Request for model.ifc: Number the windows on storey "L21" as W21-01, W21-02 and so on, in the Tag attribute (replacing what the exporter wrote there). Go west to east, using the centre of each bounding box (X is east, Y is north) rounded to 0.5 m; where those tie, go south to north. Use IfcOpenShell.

First a look at what the model holds.

```python
import ifcopenshell
import ifcopenshell.util.element
import ifcopenshell.util.placement

model = ifcopenshell.open("model.ifc")
print(model.schema)
storey = next(s for s in model.by_type("IfcBuildingStorey") if s.Name == "L21")
windows = [e for e in ifcopenshell.util.element.get_decomposition(storey) if e.is_a("IfcWindow")]
for e in sorted(windows, key=lambda e: e.id()):
    origin = ifcopenshell.util.placement.get_local_placement(e.ObjectPlacement)[:3, 3]
    print(e.id(), e.Tag, e.Name, origin.round(2) + 0.0, sep=" | ")
```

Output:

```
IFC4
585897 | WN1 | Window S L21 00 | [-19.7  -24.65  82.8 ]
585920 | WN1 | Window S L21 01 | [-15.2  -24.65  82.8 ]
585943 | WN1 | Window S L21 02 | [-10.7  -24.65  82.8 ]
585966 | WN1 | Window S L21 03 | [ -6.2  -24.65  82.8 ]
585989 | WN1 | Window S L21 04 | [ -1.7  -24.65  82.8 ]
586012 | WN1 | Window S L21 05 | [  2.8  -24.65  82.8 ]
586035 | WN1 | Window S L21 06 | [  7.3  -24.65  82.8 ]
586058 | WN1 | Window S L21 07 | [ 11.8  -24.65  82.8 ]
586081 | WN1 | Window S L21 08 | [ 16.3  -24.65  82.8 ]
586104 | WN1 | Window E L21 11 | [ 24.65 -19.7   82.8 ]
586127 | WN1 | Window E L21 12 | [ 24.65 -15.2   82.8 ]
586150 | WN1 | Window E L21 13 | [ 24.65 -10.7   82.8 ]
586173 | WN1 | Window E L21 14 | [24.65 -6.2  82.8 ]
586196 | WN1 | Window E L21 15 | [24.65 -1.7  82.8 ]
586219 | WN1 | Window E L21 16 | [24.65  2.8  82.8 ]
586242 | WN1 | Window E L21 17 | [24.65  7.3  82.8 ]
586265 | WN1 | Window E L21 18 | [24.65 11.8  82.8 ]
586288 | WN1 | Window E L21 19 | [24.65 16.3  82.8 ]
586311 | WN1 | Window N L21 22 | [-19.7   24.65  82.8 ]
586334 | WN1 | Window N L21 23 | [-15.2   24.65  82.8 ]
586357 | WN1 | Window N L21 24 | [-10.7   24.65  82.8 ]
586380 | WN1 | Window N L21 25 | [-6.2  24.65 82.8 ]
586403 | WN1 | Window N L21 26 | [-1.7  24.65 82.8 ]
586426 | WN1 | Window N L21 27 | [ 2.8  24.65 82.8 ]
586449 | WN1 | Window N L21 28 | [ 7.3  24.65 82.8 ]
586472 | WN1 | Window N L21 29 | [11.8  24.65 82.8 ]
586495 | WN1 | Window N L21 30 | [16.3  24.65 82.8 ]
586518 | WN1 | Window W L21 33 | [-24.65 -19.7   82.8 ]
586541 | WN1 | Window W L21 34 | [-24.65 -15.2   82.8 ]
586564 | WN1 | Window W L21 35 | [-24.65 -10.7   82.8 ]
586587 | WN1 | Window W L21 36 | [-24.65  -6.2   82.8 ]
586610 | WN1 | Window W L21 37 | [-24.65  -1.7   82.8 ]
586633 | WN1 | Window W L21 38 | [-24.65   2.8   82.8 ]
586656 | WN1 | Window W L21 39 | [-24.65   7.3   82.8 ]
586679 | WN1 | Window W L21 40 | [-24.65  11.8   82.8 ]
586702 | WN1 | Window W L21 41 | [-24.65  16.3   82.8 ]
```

```python
import ifcopenshell
import ifcopenshell.geom
import ifcopenshell.util.element
import ifcopenshell.util.shape

model = ifcopenshell.open("model.ifc")
settings = ifcopenshell.geom.settings()
settings.set("use-world-coords", True)


def centre(element):
    shape = ifcopenshell.geom.create_shape(settings, element)
    return ifcopenshell.util.shape.get_bbox_centroid(shape.geometry)


storey = next(s for s in model.by_type("IfcBuildingStorey") if s.Name == "L21")
windows = [e for e in ifcopenshell.util.element.get_decomposition(storey) if e.is_a("IfcWindow")]

# Insertion points can sit at a corner or the storey origin, so sort by the geometry (in metres).
centres = {e: centre(e) for e in windows}
windows.sort(key=lambda e: (round(centres[e][0] / 0.5), centres[e][1]))

for i, e in enumerate(windows, start=1):
    number = f"W21-{i:02d}"
    e.Tag = number
    print(e.id(), number)

model.write("model-out.ifc")
```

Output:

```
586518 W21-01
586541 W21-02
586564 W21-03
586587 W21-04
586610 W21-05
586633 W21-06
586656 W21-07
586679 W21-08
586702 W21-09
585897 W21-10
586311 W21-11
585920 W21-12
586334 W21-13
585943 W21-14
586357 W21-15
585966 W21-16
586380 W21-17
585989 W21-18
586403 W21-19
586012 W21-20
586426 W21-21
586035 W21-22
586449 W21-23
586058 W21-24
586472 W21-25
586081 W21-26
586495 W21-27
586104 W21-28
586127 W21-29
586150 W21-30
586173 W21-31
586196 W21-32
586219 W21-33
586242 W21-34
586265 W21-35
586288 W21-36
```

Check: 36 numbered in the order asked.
